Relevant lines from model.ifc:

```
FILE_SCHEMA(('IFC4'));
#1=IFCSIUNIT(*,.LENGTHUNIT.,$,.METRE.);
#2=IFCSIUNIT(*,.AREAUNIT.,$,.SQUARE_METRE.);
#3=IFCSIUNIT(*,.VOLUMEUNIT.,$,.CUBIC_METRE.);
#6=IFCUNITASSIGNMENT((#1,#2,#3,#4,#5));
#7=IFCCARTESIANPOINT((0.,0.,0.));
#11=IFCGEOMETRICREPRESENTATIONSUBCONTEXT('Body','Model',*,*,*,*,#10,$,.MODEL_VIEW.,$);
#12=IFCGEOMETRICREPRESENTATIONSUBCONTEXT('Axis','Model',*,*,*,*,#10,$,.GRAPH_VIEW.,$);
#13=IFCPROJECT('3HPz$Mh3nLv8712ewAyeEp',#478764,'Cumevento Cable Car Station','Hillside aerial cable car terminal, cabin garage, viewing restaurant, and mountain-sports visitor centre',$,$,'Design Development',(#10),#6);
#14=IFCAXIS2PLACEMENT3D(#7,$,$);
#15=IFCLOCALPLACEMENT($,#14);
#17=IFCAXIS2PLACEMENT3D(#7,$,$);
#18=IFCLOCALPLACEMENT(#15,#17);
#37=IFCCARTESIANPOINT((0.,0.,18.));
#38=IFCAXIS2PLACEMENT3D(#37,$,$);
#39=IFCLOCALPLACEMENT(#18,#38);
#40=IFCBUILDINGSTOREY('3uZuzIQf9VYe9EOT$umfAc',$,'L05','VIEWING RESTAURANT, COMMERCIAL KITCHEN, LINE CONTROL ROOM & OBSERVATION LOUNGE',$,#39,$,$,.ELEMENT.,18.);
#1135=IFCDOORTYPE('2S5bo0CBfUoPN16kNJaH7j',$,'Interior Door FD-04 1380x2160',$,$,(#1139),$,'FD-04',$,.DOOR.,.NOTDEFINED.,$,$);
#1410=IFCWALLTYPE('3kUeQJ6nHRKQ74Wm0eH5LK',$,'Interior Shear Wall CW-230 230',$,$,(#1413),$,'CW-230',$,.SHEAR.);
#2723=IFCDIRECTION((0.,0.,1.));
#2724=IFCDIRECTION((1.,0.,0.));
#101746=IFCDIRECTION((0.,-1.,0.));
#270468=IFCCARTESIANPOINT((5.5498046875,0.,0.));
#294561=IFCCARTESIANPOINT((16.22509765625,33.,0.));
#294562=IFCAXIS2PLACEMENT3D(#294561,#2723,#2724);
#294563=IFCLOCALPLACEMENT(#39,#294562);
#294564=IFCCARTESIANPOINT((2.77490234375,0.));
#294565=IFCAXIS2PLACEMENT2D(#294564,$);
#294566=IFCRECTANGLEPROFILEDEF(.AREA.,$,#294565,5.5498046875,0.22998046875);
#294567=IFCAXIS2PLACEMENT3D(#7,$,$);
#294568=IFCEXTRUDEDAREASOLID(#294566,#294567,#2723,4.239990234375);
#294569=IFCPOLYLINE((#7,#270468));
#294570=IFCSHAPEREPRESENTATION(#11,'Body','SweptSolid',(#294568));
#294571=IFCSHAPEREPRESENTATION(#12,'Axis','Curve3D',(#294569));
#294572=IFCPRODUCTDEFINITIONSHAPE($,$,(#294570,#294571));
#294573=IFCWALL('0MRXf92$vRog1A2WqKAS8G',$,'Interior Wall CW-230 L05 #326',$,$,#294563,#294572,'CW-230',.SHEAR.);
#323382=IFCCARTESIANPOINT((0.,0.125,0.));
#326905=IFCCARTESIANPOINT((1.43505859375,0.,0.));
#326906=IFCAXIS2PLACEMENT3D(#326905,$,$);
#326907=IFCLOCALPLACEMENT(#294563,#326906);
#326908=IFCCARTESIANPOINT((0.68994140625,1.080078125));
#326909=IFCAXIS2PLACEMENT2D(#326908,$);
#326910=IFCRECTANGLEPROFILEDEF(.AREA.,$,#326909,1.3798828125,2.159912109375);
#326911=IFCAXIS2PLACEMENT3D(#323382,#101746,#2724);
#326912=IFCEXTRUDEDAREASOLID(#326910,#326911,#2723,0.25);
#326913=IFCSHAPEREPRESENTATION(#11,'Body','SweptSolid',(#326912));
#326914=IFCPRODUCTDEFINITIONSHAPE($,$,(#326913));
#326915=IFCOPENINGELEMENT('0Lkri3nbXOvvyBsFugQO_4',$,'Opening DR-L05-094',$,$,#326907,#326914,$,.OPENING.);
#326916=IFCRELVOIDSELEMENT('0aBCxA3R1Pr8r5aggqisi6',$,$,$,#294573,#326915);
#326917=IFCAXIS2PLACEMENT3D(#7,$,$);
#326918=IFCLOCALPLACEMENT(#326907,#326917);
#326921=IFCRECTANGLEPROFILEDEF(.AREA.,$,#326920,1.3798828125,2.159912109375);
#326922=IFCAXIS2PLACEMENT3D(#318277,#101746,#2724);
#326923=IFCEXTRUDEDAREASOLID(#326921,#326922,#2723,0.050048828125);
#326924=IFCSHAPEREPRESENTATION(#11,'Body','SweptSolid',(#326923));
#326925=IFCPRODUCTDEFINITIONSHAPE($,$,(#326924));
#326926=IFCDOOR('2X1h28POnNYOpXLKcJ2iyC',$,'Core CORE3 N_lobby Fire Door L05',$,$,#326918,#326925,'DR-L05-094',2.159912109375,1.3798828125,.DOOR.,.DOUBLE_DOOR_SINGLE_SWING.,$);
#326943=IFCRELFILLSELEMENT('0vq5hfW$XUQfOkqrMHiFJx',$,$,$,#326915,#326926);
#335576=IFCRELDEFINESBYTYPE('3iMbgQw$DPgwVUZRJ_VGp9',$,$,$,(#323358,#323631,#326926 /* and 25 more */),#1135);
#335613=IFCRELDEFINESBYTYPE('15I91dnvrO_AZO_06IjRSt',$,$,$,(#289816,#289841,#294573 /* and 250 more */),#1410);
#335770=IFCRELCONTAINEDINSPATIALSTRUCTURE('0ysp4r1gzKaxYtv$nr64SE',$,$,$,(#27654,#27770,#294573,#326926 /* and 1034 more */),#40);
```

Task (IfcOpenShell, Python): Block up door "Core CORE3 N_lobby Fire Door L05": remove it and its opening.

```python
import ifcopenshell
import ifcopenshell.api.feature
import ifcopenshell.api.root
import ifcopenshell.geom
import ifcopenshell.util.shape

model = ifcopenshell.open("model.ifc")
settings = ifcopenshell.geom.settings()


def volume(element):
    """Net volume in cubic metres, openings subtracted."""
    shape = ifcopenshell.geom.create_shape(settings, element)
    return ifcopenshell.util.shape.get_volume(shape.geometry)


door = model.by_id(326926)
opening = door.FillsVoids[0].RelatingOpeningElement
wall = opening.VoidsElements[0].RelatingBuildingElement
before = volume(wall)

ifcopenshell.api.root.remove_product(model, product=door)
ifcopenshell.api.feature.remove_feature(model, feature=opening)

after = volume(wall)

print(f"wall volume {before:.3f} -> {after:.3f} m3")

model.write("model_v2.ifc")
```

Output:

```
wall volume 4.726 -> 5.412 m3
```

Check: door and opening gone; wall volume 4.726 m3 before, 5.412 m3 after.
